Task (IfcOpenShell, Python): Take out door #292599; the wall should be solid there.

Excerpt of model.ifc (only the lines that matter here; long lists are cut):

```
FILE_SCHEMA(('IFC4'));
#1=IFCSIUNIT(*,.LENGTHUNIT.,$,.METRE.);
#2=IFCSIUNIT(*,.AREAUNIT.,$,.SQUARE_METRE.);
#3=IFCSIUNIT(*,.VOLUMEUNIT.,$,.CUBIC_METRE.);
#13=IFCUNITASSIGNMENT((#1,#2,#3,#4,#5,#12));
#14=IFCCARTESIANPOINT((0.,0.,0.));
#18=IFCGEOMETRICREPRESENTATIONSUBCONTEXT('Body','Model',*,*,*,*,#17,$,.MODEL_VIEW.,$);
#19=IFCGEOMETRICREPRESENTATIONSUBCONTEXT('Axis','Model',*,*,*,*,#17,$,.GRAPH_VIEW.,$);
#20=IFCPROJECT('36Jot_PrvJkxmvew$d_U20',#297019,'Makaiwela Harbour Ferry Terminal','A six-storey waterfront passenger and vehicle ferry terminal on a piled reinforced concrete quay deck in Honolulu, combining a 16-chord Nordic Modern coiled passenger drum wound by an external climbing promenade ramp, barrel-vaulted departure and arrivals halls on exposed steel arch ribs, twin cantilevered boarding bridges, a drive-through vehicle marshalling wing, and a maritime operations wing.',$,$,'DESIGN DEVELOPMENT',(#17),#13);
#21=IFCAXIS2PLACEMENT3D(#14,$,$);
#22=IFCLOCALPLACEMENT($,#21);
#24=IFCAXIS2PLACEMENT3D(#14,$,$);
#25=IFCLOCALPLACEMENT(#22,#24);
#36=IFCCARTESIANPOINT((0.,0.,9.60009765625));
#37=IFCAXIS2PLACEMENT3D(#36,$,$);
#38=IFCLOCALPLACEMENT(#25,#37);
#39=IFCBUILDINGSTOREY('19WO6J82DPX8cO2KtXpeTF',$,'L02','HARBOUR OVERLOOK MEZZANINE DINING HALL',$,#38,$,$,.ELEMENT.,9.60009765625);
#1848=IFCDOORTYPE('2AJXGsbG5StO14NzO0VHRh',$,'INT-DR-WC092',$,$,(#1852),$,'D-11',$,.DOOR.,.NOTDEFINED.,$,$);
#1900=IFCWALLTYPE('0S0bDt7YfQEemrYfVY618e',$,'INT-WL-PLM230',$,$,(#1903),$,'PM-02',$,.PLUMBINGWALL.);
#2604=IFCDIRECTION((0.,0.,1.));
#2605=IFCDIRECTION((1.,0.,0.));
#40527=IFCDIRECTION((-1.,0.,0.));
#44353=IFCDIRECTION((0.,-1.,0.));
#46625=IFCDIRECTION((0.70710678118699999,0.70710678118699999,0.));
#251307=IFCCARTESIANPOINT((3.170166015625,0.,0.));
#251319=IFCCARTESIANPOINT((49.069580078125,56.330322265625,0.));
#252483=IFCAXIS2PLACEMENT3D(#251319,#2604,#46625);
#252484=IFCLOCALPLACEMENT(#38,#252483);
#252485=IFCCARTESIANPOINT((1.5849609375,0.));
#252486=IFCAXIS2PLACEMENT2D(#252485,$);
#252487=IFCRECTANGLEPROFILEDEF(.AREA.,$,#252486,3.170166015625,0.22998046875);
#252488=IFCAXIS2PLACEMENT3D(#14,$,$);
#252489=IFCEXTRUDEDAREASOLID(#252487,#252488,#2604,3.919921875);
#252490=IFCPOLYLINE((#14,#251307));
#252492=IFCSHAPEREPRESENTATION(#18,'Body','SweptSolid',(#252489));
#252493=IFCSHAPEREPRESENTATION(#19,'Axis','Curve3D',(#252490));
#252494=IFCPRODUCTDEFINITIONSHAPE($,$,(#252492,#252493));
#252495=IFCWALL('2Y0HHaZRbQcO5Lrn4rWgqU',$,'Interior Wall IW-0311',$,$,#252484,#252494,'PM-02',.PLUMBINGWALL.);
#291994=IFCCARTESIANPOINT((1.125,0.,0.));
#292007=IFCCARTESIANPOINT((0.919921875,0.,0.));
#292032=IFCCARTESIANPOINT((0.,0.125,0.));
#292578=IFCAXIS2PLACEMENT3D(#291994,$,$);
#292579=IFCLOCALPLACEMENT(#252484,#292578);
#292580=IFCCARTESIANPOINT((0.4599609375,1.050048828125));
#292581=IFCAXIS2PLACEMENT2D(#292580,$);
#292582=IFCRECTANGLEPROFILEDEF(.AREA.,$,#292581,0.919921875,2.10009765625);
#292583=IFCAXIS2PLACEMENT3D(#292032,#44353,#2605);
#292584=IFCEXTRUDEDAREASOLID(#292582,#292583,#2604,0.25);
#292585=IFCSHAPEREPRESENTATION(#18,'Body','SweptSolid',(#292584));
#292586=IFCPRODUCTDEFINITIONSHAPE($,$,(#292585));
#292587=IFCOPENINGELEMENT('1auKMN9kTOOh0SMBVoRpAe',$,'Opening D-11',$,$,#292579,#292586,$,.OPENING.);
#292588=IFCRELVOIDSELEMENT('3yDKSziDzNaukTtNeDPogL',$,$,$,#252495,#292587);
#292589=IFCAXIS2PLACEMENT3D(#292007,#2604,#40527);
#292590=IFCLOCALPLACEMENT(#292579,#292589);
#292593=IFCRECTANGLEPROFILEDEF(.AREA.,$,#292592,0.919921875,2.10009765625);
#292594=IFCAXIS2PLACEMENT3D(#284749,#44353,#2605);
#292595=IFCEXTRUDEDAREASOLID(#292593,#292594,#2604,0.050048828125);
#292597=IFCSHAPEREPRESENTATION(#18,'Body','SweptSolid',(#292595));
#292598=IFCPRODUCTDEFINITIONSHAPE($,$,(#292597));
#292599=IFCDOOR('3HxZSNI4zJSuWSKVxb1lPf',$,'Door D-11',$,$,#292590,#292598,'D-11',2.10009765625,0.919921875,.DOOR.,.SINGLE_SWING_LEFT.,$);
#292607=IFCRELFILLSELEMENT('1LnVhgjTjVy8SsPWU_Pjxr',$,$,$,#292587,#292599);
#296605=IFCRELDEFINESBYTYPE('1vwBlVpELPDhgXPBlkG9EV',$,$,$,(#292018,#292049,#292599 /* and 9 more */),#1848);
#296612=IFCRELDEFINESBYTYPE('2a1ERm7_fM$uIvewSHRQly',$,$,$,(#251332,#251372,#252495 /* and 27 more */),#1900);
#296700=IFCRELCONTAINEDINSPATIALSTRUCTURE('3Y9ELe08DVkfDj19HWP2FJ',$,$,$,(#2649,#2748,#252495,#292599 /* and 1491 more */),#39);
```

```python
import ifcopenshell
import ifcopenshell.api.feature
import ifcopenshell.api.root
import ifcopenshell.geom
import ifcopenshell.util.shape

model = ifcopenshell.open("model.ifc")
settings = ifcopenshell.geom.settings()


def volume(element):
    """Net volume in cubic metres, openings subtracted."""
    shape = ifcopenshell.geom.create_shape(settings, element)
    return ifcopenshell.util.shape.get_volume(shape.geometry)


door = model.by_guid("3HxZSNI4zJSuWSKVxb1lPf")
opening = door.FillsVoids[0].RelatingOpeningElement
wall = opening.VoidsElements[0].RelatingBuildingElement
before = volume(wall)

ifcopenshell.api.root.remove_product(model, product=door)
ifcopenshell.api.feature.remove_feature(model, feature=opening)

after = volume(wall)

print(f"wall volume {before:.3f} -> {after:.3f} m3")

model.write("model_v2.ifc")
```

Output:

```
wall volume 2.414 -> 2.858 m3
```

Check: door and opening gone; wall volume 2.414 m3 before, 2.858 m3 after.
